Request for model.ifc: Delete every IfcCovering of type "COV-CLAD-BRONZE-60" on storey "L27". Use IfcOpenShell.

First a look at what the model holds.

```python
import ifcopenshell
import ifcopenshell.util.element

model = ifcopenshell.open("model.ifc")
print(model.schema)
storey = next(s for s in model.by_type("IfcBuildingStorey") if s.Name == "L27")
coverings = [e for e in ifcopenshell.util.element.get_decomposition(storey) if e.is_a("IfcCovering")]
seen = {}
for e in coverings:
    element_type = ifcopenshell.util.element.get_type(e)
    name = element_type.Name if element_type not in (None, e) else None
    seen[name] = seen.get(name, 0) + 1
for name, count in sorted(seen.items(), key=str):
    print(count, "x", name)
```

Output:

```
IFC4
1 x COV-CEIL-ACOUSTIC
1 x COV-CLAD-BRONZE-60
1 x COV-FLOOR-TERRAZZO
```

```python
import ifcopenshell
import ifcopenshell.api.root
import ifcopenshell.util.element

model = ifcopenshell.open("model.ifc")

storey = next(s for s in model.by_type("IfcBuildingStorey") if s.Name == "L27")
coverings = [e for e in ifcopenshell.util.element.get_decomposition(storey) if e.is_a("IfcCovering")]
targets = [e for e in coverings if (t := ifcopenshell.util.element.get_type(e)) not in (None, e) and t.Name == "COV-CLAD-BRONZE-60"]

for e in targets:
    ifcopenshell.api.root.remove_product(model, product=e)
print(len(targets), "removed")

model.write("model_edited.ifc")
```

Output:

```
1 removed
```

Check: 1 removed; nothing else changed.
